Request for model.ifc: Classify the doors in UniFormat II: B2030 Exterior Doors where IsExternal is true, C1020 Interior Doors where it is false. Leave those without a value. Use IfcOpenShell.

First a look at what the model holds.

```python
import ifcopenshell
import ifcopenshell.util.element

model = ifcopenshell.open("model.ifc")
print(model.schema)
print("classifications:", [c.Name for c in model.by_type("IfcClassification")])
values = [ifcopenshell.util.element.get_pset(e, "Pset_DoorCommon", "IsExternal") for e in model.by_type("IfcDoor")]
for value in (True, False, None):
    print("IsExternal", value, values.count(value))
```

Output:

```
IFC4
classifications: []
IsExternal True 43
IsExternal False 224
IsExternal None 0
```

```python
import ifcopenshell
import ifcopenshell.api.classification
import ifcopenshell.util.element

model = ifcopenshell.open("model.ifc")

system = ifcopenshell.api.classification.add_classification(model, classification="UniFormat II")

doors = model.by_type("IfcDoor")
external = {e: ifcopenshell.util.element.get_pset(e, "Pset_DoorCommon", "IsExternal") for e in doors}
for flag, code, name in ((True, "B2030", "Exterior Doors"), (False, "C1020", "Interior Doors")):
    products = [e for e in doors if external[e] is flag]
    ifcopenshell.api.classification.add_reference(
        model, products=products, classification=system, identification=code, name=name
    )
    print(code, len(products))

model.write("model_updated.ifc")
```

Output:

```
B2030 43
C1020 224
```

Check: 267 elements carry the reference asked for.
